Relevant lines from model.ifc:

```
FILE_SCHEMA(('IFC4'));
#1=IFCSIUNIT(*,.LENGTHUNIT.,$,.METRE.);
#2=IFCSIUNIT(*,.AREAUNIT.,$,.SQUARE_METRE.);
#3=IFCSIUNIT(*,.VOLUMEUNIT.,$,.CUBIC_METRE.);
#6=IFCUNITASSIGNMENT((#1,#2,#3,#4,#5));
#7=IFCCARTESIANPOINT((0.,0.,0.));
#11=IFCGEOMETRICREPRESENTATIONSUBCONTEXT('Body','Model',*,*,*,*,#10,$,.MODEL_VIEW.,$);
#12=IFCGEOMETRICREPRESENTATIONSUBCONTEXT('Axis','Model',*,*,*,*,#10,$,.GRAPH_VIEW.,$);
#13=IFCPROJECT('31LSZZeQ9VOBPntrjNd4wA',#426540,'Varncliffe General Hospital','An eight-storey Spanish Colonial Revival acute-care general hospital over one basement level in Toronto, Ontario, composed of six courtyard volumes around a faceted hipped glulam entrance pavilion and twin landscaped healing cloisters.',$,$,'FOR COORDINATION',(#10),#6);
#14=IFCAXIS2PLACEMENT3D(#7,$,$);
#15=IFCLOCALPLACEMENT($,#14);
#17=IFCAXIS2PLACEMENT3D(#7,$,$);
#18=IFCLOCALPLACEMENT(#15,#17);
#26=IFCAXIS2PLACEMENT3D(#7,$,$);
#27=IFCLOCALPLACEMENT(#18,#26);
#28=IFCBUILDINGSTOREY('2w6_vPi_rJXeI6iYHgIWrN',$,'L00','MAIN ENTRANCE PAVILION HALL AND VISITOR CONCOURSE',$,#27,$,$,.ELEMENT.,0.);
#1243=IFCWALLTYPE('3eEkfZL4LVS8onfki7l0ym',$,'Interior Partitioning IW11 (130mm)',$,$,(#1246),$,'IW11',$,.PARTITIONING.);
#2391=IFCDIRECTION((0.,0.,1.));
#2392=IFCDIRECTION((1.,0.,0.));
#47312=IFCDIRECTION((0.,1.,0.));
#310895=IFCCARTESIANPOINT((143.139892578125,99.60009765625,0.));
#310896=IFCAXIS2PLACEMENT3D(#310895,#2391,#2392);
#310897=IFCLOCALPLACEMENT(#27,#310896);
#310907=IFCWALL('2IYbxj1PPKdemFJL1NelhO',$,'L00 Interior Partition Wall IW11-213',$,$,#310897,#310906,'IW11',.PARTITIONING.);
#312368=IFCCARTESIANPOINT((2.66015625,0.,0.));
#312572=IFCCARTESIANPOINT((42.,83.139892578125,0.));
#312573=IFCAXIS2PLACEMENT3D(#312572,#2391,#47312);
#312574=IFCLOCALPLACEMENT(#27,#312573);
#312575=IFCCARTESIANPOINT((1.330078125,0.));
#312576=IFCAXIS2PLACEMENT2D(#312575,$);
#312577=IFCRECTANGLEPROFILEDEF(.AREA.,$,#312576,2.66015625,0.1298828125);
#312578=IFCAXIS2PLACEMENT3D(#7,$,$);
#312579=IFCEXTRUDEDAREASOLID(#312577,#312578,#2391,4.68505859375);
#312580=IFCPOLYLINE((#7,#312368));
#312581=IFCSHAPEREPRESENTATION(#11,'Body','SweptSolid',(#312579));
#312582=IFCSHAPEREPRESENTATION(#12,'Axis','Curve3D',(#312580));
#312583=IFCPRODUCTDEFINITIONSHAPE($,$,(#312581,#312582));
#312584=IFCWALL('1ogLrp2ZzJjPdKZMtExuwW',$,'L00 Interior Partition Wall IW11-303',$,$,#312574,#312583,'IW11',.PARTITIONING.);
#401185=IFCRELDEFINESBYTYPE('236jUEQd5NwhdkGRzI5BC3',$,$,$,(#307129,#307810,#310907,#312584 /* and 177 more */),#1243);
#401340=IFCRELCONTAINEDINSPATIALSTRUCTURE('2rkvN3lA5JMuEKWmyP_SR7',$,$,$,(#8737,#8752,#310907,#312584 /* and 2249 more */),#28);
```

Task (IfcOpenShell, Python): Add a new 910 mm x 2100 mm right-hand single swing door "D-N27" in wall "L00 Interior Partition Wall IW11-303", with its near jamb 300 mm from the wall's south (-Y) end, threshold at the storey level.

```python
import numpy as np
import ifcopenshell
import ifcopenshell.api.feature
import ifcopenshell.api.geometry
import ifcopenshell.api.root
import ifcopenshell.api.spatial
import ifcopenshell.geom
import ifcopenshell.util.element
import ifcopenshell.util.placement
import ifcopenshell.util.representation
import ifcopenshell.util.shape
import ifcopenshell.util.unit

model = ifcopenshell.open("model.ifc")
unit_scale = ifcopenshell.util.unit.calculate_unit_scale(model)
settings = ifcopenshell.geom.settings()


def volume(element):
    """Net volume in cubic metres, openings subtracted."""
    shape = ifcopenshell.geom.create_shape(settings, element)
    return ifcopenshell.util.shape.get_volume(shape.geometry)


wall = model.by_guid("1ogLrp2ZzJjPdKZMtExuwW")
storey = ifcopenshell.util.element.get_container(wall, ifc_class="IfcBuildingStorey")
context = ifcopenshell.util.representation.get_context(model, "Model", "Body", "MODEL_VIEW")
before = volume(wall)

width, height, from_end, sill = 0.91, 2.1, 0.3, 0.0  # metres

# The wall runs along its own X axis, and the end named is its -X end.
wall_shape = ifcopenshell.geom.create_shape(settings, wall)
x, y, z = ifcopenshell.util.shape.get_vertices(wall_shape.geometry).T
start = x.min() + from_end
face, thickness = float(y.min()), float(y.max() - y.min())
wall_matrix = ifcopenshell.util.placement.get_local_placement(wall.ObjectPlacement)
level = ifcopenshell.util.placement.get_local_placement(storey.ObjectPlacement)[2, 3]


def in_wall(x, y):
    """Placement at x, y metres in the wall's axes, at sill height."""
    matrix = wall_matrix.copy()
    matrix[:, 3] = wall_matrix @ np.array([x / unit_scale, y / unit_scale, 0.0, 1.0])
    matrix[2, 3] = level + sill / unit_scale
    return matrix


# Opening: a box that overshoots both wall faces by 50 mm.
opening = ifcopenshell.api.root.create_entity(model, ifc_class="IfcOpeningElement", predefined_type="OPENING")
box = ifcopenshell.api.geometry.add_wall_representation(
    model, context=context, length=width, height=height, thickness=thickness + 0.1
)
ifcopenshell.api.geometry.assign_representation(model, product=opening, representation=box)
ifcopenshell.api.geometry.edit_object_placement(model, product=opening, matrix=in_wall(start, face - 0.05), is_si=False)
ifcopenshell.api.feature.add_feature(model, feature=opening, element=wall)

door = ifcopenshell.api.root.create_entity(model, ifc_class="IfcDoor", name="D-N27", predefined_type="DOOR")
door.OverallWidth, door.OverallHeight = width / unit_scale, height / unit_scale
door.OperationType = "SINGLE_SWING_RIGHT"
body = ifcopenshell.api.geometry.add_door_representation(
    model,
    context=context,
    overall_width=door.OverallWidth,
    overall_height=door.OverallHeight,
    operation_type="SINGLE_SWING_RIGHT",
    lining_properties={"LiningDepth": thickness / unit_scale, "ThresholdDepth": thickness / unit_scale},
)
ifcopenshell.api.geometry.assign_representation(model, product=door, representation=body)
ifcopenshell.api.spatial.assign_container(model, products=[door], relating_structure=storey)
ifcopenshell.api.feature.add_filling(model, opening=opening, element=door)

# The lining spans the wall, so the door starts at the wall face.
ifcopenshell.api.geometry.edit_object_placement(model, product=door, matrix=in_wall(start, face), is_si=False)

after = volume(wall)

print(f"wall volume {before:.3f} -> {after:.3f} m3")

model.write("model_v2.ifc")
```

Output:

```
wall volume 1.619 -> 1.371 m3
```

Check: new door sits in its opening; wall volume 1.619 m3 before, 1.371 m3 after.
